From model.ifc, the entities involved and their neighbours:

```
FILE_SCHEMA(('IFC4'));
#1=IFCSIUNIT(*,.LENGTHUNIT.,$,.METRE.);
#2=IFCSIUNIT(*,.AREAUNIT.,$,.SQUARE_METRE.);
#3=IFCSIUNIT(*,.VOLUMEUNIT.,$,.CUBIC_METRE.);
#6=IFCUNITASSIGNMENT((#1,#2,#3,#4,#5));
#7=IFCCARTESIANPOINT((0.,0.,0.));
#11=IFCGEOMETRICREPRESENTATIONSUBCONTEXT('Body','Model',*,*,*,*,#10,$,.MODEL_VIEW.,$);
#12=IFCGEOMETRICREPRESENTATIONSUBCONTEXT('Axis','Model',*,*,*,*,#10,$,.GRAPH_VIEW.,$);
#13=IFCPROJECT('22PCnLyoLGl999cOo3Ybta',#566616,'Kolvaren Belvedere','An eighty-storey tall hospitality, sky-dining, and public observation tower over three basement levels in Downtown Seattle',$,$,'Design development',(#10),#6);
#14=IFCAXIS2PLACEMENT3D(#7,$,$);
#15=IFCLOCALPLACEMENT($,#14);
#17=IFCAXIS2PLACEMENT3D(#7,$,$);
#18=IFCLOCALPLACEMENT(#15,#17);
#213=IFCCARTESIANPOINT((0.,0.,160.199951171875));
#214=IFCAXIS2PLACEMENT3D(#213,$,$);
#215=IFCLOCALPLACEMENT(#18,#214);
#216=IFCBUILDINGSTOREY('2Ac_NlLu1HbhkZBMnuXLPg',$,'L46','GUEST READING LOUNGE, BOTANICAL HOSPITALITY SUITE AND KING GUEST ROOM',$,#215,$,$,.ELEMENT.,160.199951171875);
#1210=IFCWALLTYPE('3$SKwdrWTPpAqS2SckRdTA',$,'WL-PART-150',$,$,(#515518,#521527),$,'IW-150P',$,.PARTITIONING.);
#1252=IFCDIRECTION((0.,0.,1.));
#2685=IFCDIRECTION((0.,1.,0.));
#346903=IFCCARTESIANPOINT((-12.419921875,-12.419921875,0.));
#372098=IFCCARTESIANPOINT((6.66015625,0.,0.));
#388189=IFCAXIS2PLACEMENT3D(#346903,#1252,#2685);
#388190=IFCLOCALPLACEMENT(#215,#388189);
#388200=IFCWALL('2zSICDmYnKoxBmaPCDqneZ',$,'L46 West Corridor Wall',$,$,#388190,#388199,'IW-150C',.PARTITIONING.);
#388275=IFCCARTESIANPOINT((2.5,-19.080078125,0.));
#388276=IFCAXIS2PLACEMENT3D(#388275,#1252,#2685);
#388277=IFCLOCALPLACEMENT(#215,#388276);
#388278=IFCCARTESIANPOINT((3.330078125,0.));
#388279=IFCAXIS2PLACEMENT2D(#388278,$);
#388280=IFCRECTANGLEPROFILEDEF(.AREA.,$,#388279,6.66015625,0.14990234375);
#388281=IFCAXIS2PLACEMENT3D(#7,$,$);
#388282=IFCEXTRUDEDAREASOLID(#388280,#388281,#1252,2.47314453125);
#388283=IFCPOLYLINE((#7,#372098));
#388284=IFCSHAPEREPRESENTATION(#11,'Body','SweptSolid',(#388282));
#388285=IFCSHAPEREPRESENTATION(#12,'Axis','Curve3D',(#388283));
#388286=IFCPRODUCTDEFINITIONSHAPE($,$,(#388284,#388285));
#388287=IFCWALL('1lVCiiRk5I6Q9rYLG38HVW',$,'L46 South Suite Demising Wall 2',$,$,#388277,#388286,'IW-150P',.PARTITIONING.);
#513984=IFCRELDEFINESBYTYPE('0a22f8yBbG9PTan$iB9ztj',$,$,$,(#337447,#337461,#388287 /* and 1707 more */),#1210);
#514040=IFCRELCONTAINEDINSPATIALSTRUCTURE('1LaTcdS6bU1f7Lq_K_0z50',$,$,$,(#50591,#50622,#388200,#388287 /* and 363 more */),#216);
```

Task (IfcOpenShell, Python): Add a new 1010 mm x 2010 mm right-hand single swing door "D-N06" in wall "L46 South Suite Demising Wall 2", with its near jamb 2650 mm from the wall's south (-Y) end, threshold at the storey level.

```python
import numpy as np
import ifcopenshell
import ifcopenshell.api.feature
import ifcopenshell.api.geometry
import ifcopenshell.api.root
import ifcopenshell.api.spatial
import ifcopenshell.geom
import ifcopenshell.util.element
import ifcopenshell.util.placement
import ifcopenshell.util.representation
import ifcopenshell.util.shape
import ifcopenshell.util.unit

model = ifcopenshell.open("model.ifc")
unit_scale = ifcopenshell.util.unit.calculate_unit_scale(model)
settings = ifcopenshell.geom.settings()


def volume(element):
    """Net volume in cubic metres, openings subtracted."""
    shape = ifcopenshell.geom.create_shape(settings, element)
    return ifcopenshell.util.shape.get_volume(shape.geometry)


wall = model.by_guid("1lVCiiRk5I6Q9rYLG38HVW")
storey = ifcopenshell.util.element.get_container(wall, ifc_class="IfcBuildingStorey")
context = ifcopenshell.util.representation.get_context(model, "Model", "Body", "MODEL_VIEW")
before = volume(wall)

width, height, from_end, sill = 1.01, 2.01, 2.65, 0.0  # metres

# The wall runs along its own X axis, and the end named is its -X end.
wall_shape = ifcopenshell.geom.create_shape(settings, wall)
x, y, z = ifcopenshell.util.shape.get_vertices(wall_shape.geometry).T
start = x.min() + from_end
face, thickness = float(y.min()), float(y.max() - y.min())
wall_matrix = ifcopenshell.util.placement.get_local_placement(wall.ObjectPlacement)
level = ifcopenshell.util.placement.get_local_placement(storey.ObjectPlacement)[2, 3]


def in_wall(x, y):
    """Placement at x, y metres in the wall's axes, at sill height."""
    matrix = wall_matrix.copy()
    matrix[:, 3] = wall_matrix @ np.array([x / unit_scale, y / unit_scale, 0.0, 1.0])
    matrix[2, 3] = level + sill / unit_scale
    return matrix


# Opening: a box that overshoots both wall faces by 50 mm.
opening = ifcopenshell.api.root.create_entity(model, ifc_class="IfcOpeningElement", predefined_type="OPENING")
box = ifcopenshell.api.geometry.add_wall_representation(
    model, context=context, length=width, height=height, thickness=thickness + 0.1
)
ifcopenshell.api.geometry.assign_representation(model, product=opening, representation=box)
ifcopenshell.api.geometry.edit_object_placement(model, product=opening, matrix=in_wall(start, face - 0.05), is_si=False)
ifcopenshell.api.feature.add_feature(model, feature=opening, element=wall)

door = ifcopenshell.api.root.create_entity(model, ifc_class="IfcDoor", name="D-N06", predefined_type="DOOR")
door.OverallWidth, door.OverallHeight = width / unit_scale, height / unit_scale
door.OperationType = "SINGLE_SWING_RIGHT"
body = ifcopenshell.api.geometry.add_door_representation(
    model,
    context=context,
    overall_width=door.OverallWidth,
    overall_height=door.OverallHeight,
    operation_type="SINGLE_SWING_RIGHT",
    lining_properties={"LiningDepth": thickness / unit_scale, "ThresholdDepth": thickness / unit_scale},
)
ifcopenshell.api.geometry.assign_representation(model, product=door, representation=body)
ifcopenshell.api.spatial.assign_container(model, products=[door], relating_structure=storey)
ifcopenshell.api.feature.add_filling(model, opening=opening, element=door)

# The lining spans the wall, so the door starts at the wall face.
ifcopenshell.api.geometry.edit_object_placement(model, product=door, matrix=in_wall(start, face), is_si=False)

after = volume(wall)

print(f"wall volume {before:.3f} -> {after:.3f} m3")

model.write("model_rev.ifc")
```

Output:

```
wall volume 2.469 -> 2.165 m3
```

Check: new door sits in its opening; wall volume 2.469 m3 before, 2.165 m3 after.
